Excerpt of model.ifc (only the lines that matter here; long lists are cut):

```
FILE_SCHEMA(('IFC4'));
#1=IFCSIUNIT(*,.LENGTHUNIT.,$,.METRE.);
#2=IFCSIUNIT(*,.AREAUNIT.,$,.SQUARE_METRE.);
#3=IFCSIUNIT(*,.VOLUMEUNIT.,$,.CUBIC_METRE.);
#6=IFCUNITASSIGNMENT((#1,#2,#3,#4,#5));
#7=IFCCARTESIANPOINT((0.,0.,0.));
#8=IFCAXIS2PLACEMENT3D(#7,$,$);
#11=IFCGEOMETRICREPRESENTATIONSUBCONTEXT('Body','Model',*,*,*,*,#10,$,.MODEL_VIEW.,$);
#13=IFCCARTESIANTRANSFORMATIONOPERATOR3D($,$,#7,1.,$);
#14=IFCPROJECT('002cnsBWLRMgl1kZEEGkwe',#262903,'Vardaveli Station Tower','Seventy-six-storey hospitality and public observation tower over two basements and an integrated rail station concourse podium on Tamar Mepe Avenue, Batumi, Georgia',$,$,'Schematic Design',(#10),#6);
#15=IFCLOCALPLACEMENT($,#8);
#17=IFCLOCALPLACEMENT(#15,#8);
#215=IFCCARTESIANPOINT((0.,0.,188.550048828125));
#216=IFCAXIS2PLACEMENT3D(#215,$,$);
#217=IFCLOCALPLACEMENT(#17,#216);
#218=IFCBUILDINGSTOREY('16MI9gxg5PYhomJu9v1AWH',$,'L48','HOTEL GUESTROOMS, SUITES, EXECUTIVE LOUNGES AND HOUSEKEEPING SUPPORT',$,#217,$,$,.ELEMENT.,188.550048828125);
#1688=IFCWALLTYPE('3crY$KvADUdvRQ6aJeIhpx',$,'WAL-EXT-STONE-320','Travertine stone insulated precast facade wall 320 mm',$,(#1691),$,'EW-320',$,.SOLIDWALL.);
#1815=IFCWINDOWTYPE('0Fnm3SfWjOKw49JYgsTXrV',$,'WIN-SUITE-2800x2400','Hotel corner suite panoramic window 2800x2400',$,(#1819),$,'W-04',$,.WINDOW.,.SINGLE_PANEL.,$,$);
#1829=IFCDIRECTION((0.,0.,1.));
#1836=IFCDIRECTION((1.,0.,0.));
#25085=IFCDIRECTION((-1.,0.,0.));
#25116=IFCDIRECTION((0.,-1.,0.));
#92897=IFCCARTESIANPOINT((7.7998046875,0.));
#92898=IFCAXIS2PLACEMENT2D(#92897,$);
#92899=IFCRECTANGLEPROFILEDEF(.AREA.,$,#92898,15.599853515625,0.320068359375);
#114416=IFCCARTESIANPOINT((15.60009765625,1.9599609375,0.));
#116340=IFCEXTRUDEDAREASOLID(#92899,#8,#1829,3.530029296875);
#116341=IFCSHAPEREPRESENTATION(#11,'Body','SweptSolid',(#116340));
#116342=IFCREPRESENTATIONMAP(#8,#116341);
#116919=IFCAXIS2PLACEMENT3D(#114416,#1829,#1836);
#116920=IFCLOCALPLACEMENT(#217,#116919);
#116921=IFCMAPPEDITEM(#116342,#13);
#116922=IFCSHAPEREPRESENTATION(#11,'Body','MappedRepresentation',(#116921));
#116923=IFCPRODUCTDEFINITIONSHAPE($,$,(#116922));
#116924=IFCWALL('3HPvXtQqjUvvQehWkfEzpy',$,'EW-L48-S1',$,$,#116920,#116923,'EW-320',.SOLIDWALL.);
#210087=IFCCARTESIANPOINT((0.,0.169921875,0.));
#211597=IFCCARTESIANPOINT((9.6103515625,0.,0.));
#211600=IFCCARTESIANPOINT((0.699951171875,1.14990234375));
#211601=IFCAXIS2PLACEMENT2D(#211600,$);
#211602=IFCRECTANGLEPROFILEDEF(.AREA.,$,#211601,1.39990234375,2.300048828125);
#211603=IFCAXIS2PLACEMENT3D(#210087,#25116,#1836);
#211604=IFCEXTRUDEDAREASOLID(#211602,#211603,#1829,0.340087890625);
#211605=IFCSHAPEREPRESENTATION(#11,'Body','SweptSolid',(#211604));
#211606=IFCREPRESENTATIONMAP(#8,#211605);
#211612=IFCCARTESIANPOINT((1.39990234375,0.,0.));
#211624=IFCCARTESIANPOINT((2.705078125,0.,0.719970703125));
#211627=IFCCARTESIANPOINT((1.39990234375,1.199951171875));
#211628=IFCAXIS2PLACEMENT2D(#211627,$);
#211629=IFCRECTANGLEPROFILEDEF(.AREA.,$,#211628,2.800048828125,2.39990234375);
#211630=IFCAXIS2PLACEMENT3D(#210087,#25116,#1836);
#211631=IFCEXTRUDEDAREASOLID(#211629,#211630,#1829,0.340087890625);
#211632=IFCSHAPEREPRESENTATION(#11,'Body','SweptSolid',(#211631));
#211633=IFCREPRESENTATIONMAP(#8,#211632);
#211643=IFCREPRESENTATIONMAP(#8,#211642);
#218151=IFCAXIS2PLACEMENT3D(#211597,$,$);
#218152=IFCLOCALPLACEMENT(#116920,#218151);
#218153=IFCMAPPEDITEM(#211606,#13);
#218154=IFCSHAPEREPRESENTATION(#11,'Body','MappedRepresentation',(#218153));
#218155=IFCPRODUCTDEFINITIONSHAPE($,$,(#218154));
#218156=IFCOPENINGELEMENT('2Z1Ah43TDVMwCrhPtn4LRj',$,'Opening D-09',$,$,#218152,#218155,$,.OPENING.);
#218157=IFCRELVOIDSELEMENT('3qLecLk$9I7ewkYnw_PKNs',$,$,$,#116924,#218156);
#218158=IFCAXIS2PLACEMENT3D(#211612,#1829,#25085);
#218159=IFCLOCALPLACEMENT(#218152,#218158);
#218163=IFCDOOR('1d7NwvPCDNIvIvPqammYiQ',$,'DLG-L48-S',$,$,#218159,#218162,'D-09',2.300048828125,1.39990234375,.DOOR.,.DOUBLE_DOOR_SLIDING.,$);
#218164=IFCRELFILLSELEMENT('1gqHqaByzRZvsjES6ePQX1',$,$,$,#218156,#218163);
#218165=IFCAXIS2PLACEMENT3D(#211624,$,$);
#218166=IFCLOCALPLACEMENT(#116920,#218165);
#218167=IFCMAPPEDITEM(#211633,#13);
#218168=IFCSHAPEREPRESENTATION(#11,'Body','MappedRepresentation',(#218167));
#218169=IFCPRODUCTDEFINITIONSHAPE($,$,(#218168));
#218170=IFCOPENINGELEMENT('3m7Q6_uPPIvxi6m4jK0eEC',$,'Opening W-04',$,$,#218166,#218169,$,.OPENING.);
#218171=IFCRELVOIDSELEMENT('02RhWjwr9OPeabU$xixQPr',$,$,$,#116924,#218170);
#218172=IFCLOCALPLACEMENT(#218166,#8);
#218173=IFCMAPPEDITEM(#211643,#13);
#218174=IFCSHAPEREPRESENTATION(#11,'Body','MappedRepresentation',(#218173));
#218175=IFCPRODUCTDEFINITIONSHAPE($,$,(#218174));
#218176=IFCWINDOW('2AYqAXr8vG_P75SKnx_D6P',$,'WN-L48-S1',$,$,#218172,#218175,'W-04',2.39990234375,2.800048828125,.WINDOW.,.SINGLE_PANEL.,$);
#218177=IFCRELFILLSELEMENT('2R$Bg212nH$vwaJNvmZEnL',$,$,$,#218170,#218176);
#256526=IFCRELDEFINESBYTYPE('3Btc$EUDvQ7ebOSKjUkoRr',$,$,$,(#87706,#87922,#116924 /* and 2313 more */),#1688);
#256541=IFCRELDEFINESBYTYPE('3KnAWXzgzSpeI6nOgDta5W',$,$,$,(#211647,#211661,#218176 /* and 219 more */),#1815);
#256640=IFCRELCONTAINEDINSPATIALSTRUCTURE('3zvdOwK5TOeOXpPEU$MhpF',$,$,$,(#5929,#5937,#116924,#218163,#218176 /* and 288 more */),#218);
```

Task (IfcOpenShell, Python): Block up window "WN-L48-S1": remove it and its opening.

```python
import ifcopenshell
import ifcopenshell.api.feature
import ifcopenshell.api.root
import ifcopenshell.geom
import ifcopenshell.util.shape

model = ifcopenshell.open("model.ifc")
settings = ifcopenshell.geom.settings()


def volume(element):
    """Net volume in cubic metres, openings subtracted."""
    shape = ifcopenshell.geom.create_shape(settings, element)
    return ifcopenshell.util.shape.get_volume(shape.geometry)


window = model.by_guid("2AYqAXr8vG_P75SKnx_D6P")
opening = window.FillsVoids[0].RelatingOpeningElement
wall = opening.VoidsElements[0].RelatingBuildingElement
before = volume(wall)

ifcopenshell.api.root.remove_product(model, product=window)
ifcopenshell.api.feature.remove_feature(model, feature=opening)

after = volume(wall)

print(f"wall volume {before:.3f} -> {after:.3f} m3")

model.write("model_updated.ifc")
```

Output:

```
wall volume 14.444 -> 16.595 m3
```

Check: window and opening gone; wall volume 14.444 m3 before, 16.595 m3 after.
